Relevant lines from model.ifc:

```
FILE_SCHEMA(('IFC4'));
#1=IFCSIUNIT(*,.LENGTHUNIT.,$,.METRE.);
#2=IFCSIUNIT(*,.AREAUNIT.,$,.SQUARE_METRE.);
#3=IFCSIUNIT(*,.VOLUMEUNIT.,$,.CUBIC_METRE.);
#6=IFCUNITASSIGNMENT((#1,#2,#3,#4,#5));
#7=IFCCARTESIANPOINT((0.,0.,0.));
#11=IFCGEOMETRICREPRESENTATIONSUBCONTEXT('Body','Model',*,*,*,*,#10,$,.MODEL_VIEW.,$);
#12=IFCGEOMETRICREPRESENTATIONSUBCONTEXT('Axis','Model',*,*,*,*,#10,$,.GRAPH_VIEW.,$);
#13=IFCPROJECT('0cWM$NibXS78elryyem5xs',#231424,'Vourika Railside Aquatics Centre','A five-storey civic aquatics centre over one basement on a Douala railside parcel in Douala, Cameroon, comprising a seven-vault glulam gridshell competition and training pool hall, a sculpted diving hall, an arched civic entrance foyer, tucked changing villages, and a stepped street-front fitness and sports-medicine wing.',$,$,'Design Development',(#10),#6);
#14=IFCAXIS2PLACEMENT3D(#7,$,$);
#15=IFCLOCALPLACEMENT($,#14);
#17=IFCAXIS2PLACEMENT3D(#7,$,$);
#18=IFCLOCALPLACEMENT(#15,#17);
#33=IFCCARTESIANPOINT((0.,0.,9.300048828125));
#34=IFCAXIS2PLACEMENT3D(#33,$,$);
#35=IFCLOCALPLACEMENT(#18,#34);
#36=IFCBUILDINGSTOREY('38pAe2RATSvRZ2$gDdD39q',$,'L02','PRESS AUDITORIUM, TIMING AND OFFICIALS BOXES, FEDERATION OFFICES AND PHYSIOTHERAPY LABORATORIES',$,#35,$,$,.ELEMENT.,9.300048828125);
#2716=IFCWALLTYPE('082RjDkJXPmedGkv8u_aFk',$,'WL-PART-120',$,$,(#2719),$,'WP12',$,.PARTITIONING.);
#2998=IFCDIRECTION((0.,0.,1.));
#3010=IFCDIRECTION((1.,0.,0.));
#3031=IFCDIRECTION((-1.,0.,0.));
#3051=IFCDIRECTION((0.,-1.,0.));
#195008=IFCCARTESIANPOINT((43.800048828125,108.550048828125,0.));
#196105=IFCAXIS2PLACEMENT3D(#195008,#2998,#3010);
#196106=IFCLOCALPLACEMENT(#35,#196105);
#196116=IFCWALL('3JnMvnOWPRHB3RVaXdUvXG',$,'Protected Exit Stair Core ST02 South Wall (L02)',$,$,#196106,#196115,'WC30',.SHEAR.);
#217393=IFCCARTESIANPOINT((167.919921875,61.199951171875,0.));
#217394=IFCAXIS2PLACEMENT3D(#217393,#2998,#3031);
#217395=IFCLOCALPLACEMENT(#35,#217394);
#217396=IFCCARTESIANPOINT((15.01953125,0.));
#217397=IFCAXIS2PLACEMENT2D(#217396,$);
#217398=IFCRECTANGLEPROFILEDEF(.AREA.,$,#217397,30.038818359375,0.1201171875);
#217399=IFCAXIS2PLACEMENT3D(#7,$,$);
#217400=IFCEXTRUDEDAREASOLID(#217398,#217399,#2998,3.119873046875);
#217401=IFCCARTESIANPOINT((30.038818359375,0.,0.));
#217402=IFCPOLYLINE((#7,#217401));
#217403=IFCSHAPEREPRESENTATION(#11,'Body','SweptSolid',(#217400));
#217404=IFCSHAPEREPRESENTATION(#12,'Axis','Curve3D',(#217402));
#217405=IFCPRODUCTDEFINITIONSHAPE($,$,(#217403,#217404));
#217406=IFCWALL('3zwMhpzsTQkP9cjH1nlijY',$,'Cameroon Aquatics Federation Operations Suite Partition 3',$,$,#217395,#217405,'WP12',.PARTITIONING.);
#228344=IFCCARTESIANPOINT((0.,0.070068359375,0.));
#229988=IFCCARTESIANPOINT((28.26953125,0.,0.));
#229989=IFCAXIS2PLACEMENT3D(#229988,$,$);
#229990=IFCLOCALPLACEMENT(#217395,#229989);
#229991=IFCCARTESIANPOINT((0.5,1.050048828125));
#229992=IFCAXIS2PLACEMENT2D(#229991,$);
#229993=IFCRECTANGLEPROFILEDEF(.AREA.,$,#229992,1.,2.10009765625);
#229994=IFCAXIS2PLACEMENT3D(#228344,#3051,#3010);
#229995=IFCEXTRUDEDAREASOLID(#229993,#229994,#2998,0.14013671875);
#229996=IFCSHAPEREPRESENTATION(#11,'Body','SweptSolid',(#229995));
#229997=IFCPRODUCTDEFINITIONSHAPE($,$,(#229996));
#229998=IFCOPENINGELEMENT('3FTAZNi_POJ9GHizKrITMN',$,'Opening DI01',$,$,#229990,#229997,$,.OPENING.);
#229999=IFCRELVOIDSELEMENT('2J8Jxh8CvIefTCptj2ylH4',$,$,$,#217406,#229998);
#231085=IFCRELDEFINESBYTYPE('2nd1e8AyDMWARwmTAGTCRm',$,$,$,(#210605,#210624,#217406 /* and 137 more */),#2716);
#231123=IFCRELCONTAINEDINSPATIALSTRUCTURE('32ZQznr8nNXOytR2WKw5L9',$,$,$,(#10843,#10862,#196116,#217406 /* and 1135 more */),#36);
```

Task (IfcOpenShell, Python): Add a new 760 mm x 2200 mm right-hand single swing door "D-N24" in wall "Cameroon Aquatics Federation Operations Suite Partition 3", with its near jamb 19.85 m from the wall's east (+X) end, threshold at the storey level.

```python
import numpy as np
import ifcopenshell
import ifcopenshell.api.feature
import ifcopenshell.api.geometry
import ifcopenshell.api.root
import ifcopenshell.api.spatial
import ifcopenshell.geom
import ifcopenshell.util.element
import ifcopenshell.util.placement
import ifcopenshell.util.representation
import ifcopenshell.util.shape
import ifcopenshell.util.unit

model = ifcopenshell.open("model.ifc")
unit_scale = ifcopenshell.util.unit.calculate_unit_scale(model)
settings = ifcopenshell.geom.settings()


def volume(element):
    """Net volume in cubic metres, openings subtracted."""
    shape = ifcopenshell.geom.create_shape(settings, element)
    return ifcopenshell.util.shape.get_volume(shape.geometry)


wall = model.by_id(217406)
storey = ifcopenshell.util.element.get_container(wall, ifc_class="IfcBuildingStorey")
context = ifcopenshell.util.representation.get_context(model, "Model", "Body", "MODEL_VIEW")
before = volume(wall)

width, height, from_end, sill = 0.76, 2.2, 19.85, 0.0  # metres

# The wall runs along its own X axis, and the end named is its -X end.
wall_shape = ifcopenshell.geom.create_shape(settings, wall)
x, y, z = ifcopenshell.util.shape.get_vertices(wall_shape.geometry).T
start = x.min() + from_end
face, thickness = float(y.min()), float(y.max() - y.min())
wall_matrix = ifcopenshell.util.placement.get_local_placement(wall.ObjectPlacement)
level = ifcopenshell.util.placement.get_local_placement(storey.ObjectPlacement)[2, 3]


def in_wall(x, y):
    """Placement at x, y metres in the wall's axes, at sill height."""
    matrix = wall_matrix.copy()
    matrix[:, 3] = wall_matrix @ np.array([x / unit_scale, y / unit_scale, 0.0, 1.0])
    matrix[2, 3] = level + sill / unit_scale
    return matrix


# Opening: a box that overshoots both wall faces by 50 mm.
opening = ifcopenshell.api.root.create_entity(model, ifc_class="IfcOpeningElement", predefined_type="OPENING")
box = ifcopenshell.api.geometry.add_wall_representation(
    model, context=context, length=width, height=height, thickness=thickness + 0.1
)
ifcopenshell.api.geometry.assign_representation(model, product=opening, representation=box)
ifcopenshell.api.geometry.edit_object_placement(model, product=opening, matrix=in_wall(start, face - 0.05), is_si=False)
ifcopenshell.api.feature.add_feature(model, feature=opening, element=wall)

door = ifcopenshell.api.root.create_entity(model, ifc_class="IfcDoor", name="D-N24", predefined_type="DOOR")
door.OverallWidth, door.OverallHeight = width / unit_scale, height / unit_scale
door.OperationType = "SINGLE_SWING_RIGHT"
body = ifcopenshell.api.geometry.add_door_representation(
    model,
    context=context,
    overall_width=door.OverallWidth,
    overall_height=door.OverallHeight,
    operation_type="SINGLE_SWING_RIGHT",
    lining_properties={"LiningDepth": thickness / unit_scale, "ThresholdDepth": thickness / unit_scale},
)
ifcopenshell.api.geometry.assign_representation(model, product=door, representation=body)
ifcopenshell.api.spatial.assign_container(model, products=[door], relating_structure=storey)
ifcopenshell.api.feature.add_filling(model, opening=opening, element=door)

# The lining spans the wall, so the door starts at the wall face.
ifcopenshell.api.geometry.edit_object_placement(model, product=door, matrix=in_wall(start, face), is_si=False)

after = volume(wall)

print(f"wall volume {before:.3f} -> {after:.3f} m3")

model.write("model-out.ifc")
```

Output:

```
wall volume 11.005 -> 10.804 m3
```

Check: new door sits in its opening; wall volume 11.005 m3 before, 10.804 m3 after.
